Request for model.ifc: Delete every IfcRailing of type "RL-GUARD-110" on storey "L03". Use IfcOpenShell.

First a look at what the model holds.

```python
import ifcopenshell
import ifcopenshell.util.element

model = ifcopenshell.open("model.ifc")
print(model.schema)
storey = next(s for s in model.by_type("IfcBuildingStorey") if s.Name == "L03")
railings = [e for e in ifcopenshell.util.element.get_decomposition(storey) if e.is_a("IfcRailing")]
seen = {}
for e in railings:
    element_type = ifcopenshell.util.element.get_type(e)
    name = element_type.Name if element_type not in (None, e) else None
    seen[name] = seen.get(name, 0) + 1
for name, count in sorted(seen.items(), key=str):
    print(count, "x", name)
```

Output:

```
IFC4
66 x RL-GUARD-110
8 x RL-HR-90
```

```python
import ifcopenshell
import ifcopenshell.api.root
import ifcopenshell.util.element

model = ifcopenshell.open("model.ifc")

storey = next(s for s in model.by_type("IfcBuildingStorey") if s.Name == "L03")
railings = [e for e in ifcopenshell.util.element.get_decomposition(storey) if e.is_a("IfcRailing")]
targets = [e for e in railings if (t := ifcopenshell.util.element.get_type(e)) not in (None, e) and t.Name == "RL-GUARD-110"]

for e in targets:
    ifcopenshell.api.root.remove_product(model, product=e)
print(len(targets), "removed")

model.write("model_edited.ifc")
```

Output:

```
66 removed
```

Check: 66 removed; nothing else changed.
